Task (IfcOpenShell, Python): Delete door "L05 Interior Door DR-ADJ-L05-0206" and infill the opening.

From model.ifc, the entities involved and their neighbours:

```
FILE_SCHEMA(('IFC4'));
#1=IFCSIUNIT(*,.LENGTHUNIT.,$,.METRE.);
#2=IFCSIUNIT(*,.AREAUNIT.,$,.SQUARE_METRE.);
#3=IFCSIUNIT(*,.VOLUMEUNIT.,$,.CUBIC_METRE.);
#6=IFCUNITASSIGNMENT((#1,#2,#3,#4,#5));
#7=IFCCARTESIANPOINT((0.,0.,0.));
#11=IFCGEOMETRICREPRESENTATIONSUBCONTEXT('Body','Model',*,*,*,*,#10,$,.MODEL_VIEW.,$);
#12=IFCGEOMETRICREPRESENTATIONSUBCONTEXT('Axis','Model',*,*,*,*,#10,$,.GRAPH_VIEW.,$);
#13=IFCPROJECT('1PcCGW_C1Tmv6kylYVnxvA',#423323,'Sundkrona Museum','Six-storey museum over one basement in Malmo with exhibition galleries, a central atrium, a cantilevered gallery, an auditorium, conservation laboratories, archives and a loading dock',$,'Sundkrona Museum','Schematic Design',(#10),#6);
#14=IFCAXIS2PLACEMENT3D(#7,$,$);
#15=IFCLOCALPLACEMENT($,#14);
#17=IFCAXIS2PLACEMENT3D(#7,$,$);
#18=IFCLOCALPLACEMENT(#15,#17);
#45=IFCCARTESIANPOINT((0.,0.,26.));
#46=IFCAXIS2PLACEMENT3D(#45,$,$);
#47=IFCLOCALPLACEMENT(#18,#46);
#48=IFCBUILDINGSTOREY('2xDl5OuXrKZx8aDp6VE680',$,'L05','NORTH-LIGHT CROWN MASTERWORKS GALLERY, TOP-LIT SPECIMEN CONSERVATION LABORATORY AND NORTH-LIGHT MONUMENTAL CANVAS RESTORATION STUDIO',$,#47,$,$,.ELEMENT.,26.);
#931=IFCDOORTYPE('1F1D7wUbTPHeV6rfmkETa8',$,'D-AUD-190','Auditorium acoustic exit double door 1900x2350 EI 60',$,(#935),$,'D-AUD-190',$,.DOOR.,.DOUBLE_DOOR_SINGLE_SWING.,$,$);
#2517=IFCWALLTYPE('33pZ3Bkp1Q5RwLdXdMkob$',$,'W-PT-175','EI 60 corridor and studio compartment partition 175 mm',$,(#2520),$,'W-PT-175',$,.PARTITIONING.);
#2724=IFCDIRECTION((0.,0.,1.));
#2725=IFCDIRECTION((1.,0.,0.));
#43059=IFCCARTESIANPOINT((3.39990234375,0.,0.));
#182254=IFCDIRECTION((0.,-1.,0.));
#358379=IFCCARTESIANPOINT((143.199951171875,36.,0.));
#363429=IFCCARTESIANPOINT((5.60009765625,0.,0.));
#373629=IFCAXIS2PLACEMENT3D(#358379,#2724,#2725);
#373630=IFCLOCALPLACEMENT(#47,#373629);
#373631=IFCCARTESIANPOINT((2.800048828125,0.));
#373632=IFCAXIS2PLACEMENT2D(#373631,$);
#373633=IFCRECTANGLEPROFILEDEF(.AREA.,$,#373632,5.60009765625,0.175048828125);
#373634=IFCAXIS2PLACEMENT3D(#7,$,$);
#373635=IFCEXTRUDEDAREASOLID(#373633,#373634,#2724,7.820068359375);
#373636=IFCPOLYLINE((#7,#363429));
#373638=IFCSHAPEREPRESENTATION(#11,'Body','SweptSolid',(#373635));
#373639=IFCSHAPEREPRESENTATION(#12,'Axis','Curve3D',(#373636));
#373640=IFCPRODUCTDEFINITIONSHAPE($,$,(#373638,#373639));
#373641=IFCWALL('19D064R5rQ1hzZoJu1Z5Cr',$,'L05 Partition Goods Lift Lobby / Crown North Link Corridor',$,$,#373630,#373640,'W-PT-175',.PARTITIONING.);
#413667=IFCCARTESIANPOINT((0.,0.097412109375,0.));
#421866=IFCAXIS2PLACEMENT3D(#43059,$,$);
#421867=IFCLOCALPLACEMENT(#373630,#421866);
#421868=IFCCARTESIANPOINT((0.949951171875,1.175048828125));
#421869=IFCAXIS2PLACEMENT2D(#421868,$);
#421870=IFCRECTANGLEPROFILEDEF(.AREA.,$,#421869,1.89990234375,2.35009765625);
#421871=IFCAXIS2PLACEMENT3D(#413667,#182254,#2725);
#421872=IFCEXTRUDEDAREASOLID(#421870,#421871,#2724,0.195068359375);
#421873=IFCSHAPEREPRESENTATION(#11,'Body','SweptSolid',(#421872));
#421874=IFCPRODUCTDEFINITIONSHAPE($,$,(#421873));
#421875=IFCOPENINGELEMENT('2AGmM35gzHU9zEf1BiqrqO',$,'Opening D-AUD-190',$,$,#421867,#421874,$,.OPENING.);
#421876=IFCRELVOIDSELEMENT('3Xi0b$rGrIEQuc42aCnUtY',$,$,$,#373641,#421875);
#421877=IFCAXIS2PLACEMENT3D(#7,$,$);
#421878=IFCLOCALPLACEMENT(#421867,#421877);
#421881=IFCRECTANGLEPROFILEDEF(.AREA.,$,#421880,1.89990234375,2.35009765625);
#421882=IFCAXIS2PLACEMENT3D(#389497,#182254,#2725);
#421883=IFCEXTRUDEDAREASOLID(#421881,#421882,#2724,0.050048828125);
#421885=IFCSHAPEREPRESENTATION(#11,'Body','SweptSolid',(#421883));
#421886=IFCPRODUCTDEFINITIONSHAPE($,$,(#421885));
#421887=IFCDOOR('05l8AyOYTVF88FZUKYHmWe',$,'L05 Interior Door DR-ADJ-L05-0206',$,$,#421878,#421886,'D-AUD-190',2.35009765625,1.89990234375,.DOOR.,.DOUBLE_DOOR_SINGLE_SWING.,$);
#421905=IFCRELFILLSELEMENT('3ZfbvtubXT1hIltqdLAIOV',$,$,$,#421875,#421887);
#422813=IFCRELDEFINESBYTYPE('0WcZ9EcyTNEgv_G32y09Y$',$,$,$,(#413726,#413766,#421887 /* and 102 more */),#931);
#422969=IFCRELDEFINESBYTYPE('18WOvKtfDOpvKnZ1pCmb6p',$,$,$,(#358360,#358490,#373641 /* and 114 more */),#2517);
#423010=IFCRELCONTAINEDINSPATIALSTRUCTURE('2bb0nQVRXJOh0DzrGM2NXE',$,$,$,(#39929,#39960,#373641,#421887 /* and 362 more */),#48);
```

```python
import ifcopenshell
import ifcopenshell.api.feature
import ifcopenshell.api.root
import ifcopenshell.geom
import ifcopenshell.util.shape

model = ifcopenshell.open("model.ifc")
settings = ifcopenshell.geom.settings()


def volume(element):
    """Net volume in cubic metres, openings subtracted."""
    shape = ifcopenshell.geom.create_shape(settings, element)
    return ifcopenshell.util.shape.get_volume(shape.geometry)


door = model.by_id(421887)
opening = door.FillsVoids[0].RelatingOpeningElement
wall = opening.VoidsElements[0].RelatingBuildingElement
before = volume(wall)

ifcopenshell.api.root.remove_product(model, product=door)
ifcopenshell.api.feature.remove_feature(model, feature=opening)

after = volume(wall)

print(f"wall volume {before:.3f} -> {after:.3f} m3")

model.write("model-out.ifc")
```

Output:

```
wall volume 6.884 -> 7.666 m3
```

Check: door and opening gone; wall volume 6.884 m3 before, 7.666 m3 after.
